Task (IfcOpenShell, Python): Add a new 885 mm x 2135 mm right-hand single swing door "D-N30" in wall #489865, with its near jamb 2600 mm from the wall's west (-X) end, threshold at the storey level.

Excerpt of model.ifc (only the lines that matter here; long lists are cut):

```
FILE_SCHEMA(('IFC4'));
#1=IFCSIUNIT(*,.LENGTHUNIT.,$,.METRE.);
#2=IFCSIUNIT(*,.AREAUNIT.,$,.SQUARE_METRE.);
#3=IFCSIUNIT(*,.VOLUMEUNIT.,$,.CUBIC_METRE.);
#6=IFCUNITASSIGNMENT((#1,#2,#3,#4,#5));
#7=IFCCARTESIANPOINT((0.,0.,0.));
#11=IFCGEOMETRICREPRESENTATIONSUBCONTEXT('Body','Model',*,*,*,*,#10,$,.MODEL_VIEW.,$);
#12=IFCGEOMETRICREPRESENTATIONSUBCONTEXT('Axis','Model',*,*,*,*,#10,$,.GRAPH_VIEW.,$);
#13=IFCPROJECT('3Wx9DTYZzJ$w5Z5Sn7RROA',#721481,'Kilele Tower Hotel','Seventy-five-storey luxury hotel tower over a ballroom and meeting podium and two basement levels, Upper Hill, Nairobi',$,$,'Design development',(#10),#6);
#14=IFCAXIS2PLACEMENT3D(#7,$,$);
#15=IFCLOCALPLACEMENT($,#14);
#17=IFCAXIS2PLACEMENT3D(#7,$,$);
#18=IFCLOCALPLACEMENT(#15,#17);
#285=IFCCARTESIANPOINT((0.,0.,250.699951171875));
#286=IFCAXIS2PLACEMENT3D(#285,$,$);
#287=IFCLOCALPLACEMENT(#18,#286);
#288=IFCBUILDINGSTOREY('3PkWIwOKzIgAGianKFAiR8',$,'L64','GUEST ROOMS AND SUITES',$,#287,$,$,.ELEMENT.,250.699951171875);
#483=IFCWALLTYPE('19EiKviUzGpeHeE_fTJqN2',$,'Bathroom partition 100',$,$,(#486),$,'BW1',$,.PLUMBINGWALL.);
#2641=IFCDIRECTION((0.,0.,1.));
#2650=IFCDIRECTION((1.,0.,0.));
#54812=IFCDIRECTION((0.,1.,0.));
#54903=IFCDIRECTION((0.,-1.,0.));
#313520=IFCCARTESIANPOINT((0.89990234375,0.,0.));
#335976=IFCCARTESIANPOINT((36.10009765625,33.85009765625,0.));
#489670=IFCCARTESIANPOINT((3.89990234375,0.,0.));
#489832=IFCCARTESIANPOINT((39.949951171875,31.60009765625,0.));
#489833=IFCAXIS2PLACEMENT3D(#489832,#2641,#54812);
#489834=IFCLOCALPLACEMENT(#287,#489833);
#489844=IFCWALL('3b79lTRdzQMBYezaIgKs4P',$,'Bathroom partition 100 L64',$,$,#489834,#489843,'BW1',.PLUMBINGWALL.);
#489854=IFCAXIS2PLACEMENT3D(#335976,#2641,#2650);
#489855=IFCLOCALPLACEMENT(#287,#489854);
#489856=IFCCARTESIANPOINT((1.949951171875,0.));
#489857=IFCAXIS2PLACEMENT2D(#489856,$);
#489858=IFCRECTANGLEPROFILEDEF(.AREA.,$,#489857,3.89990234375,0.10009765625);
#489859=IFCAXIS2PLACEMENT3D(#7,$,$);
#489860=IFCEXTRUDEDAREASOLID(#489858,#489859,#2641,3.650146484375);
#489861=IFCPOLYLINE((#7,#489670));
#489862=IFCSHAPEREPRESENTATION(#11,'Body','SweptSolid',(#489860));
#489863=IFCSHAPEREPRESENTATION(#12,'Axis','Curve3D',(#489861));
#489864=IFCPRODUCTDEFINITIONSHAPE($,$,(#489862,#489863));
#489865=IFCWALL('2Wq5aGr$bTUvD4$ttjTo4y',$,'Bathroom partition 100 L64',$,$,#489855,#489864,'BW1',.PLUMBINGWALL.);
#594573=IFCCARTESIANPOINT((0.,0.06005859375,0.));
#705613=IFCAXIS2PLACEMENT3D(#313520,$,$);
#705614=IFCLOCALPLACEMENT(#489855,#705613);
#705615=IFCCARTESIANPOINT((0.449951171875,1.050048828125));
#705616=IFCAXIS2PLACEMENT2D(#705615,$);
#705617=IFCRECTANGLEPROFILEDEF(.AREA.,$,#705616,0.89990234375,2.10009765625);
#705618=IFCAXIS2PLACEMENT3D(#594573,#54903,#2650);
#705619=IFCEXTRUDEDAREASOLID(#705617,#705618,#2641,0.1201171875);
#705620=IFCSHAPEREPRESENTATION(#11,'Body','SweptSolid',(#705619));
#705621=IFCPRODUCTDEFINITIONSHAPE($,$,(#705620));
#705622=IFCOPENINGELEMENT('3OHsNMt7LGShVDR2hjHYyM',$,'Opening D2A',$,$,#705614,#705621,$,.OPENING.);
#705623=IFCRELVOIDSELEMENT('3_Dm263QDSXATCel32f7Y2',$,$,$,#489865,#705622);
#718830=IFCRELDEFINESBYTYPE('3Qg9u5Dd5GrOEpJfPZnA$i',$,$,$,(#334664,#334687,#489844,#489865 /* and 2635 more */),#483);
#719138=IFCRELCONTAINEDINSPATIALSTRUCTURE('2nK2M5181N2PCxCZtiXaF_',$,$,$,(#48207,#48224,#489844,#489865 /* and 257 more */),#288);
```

```python
import numpy as np
import ifcopenshell
import ifcopenshell.api.feature
import ifcopenshell.api.geometry
import ifcopenshell.api.root
import ifcopenshell.api.spatial
import ifcopenshell.geom
import ifcopenshell.util.element
import ifcopenshell.util.placement
import ifcopenshell.util.representation
import ifcopenshell.util.shape
import ifcopenshell.util.unit

model = ifcopenshell.open("model.ifc")
unit_scale = ifcopenshell.util.unit.calculate_unit_scale(model)
settings = ifcopenshell.geom.settings()


def volume(element):
    """Net volume in cubic metres, openings subtracted."""
    shape = ifcopenshell.geom.create_shape(settings, element)
    return ifcopenshell.util.shape.get_volume(shape.geometry)


wall = model.by_guid("2Wq5aGr$bTUvD4$ttjTo4y")
storey = ifcopenshell.util.element.get_container(wall, ifc_class="IfcBuildingStorey")
context = ifcopenshell.util.representation.get_context(model, "Model", "Body", "MODEL_VIEW")
before = volume(wall)

width, height, from_end, sill = 0.885, 2.135, 2.6, 0.0  # metres

# The wall runs along its own X axis, and the end named is its -X end.
wall_shape = ifcopenshell.geom.create_shape(settings, wall)
x, y, z = ifcopenshell.util.shape.get_vertices(wall_shape.geometry).T
start = x.min() + from_end
face, thickness = float(y.min()), float(y.max() - y.min())
wall_matrix = ifcopenshell.util.placement.get_local_placement(wall.ObjectPlacement)
level = ifcopenshell.util.placement.get_local_placement(storey.ObjectPlacement)[2, 3]


def in_wall(x, y):
    """Placement at x, y metres in the wall's axes, at sill height."""
    matrix = wall_matrix.copy()
    matrix[:, 3] = wall_matrix @ np.array([x / unit_scale, y / unit_scale, 0.0, 1.0])
    matrix[2, 3] = level + sill / unit_scale
    return matrix


# Opening: a box that overshoots both wall faces by 50 mm.
opening = ifcopenshell.api.root.create_entity(model, ifc_class="IfcOpeningElement", predefined_type="OPENING")
box = ifcopenshell.api.geometry.add_wall_representation(
    model, context=context, length=width, height=height, thickness=thickness + 0.1
)
ifcopenshell.api.geometry.assign_representation(model, product=opening, representation=box)
ifcopenshell.api.geometry.edit_object_placement(model, product=opening, matrix=in_wall(start, face - 0.05), is_si=False)
ifcopenshell.api.feature.add_feature(model, feature=opening, element=wall)

door = ifcopenshell.api.root.create_entity(model, ifc_class="IfcDoor", name="D-N30", predefined_type="DOOR")
door.OverallWidth, door.OverallHeight = width / unit_scale, height / unit_scale
door.OperationType = "SINGLE_SWING_RIGHT"
body = ifcopenshell.api.geometry.add_door_representation(
    model,
    context=context,
    overall_width=door.OverallWidth,
    overall_height=door.OverallHeight,
    operation_type="SINGLE_SWING_RIGHT",
    lining_properties={"LiningDepth": thickness / unit_scale, "ThresholdDepth": thickness / unit_scale},
)
ifcopenshell.api.geometry.assign_representation(model, product=door, representation=body)
ifcopenshell.api.spatial.assign_container(model, products=[door], relating_structure=storey)
ifcopenshell.api.feature.add_filling(model, opening=opening, element=door)

# The lining spans the wall, so the door starts at the wall face.
ifcopenshell.api.geometry.edit_object_placement(model, product=door, matrix=in_wall(start, face), is_si=False)

after = volume(wall)

print(f"wall volume {before:.3f} -> {after:.3f} m3")

model.write("model-out.ifc")
```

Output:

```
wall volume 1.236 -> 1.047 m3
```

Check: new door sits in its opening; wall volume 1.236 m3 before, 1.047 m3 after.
